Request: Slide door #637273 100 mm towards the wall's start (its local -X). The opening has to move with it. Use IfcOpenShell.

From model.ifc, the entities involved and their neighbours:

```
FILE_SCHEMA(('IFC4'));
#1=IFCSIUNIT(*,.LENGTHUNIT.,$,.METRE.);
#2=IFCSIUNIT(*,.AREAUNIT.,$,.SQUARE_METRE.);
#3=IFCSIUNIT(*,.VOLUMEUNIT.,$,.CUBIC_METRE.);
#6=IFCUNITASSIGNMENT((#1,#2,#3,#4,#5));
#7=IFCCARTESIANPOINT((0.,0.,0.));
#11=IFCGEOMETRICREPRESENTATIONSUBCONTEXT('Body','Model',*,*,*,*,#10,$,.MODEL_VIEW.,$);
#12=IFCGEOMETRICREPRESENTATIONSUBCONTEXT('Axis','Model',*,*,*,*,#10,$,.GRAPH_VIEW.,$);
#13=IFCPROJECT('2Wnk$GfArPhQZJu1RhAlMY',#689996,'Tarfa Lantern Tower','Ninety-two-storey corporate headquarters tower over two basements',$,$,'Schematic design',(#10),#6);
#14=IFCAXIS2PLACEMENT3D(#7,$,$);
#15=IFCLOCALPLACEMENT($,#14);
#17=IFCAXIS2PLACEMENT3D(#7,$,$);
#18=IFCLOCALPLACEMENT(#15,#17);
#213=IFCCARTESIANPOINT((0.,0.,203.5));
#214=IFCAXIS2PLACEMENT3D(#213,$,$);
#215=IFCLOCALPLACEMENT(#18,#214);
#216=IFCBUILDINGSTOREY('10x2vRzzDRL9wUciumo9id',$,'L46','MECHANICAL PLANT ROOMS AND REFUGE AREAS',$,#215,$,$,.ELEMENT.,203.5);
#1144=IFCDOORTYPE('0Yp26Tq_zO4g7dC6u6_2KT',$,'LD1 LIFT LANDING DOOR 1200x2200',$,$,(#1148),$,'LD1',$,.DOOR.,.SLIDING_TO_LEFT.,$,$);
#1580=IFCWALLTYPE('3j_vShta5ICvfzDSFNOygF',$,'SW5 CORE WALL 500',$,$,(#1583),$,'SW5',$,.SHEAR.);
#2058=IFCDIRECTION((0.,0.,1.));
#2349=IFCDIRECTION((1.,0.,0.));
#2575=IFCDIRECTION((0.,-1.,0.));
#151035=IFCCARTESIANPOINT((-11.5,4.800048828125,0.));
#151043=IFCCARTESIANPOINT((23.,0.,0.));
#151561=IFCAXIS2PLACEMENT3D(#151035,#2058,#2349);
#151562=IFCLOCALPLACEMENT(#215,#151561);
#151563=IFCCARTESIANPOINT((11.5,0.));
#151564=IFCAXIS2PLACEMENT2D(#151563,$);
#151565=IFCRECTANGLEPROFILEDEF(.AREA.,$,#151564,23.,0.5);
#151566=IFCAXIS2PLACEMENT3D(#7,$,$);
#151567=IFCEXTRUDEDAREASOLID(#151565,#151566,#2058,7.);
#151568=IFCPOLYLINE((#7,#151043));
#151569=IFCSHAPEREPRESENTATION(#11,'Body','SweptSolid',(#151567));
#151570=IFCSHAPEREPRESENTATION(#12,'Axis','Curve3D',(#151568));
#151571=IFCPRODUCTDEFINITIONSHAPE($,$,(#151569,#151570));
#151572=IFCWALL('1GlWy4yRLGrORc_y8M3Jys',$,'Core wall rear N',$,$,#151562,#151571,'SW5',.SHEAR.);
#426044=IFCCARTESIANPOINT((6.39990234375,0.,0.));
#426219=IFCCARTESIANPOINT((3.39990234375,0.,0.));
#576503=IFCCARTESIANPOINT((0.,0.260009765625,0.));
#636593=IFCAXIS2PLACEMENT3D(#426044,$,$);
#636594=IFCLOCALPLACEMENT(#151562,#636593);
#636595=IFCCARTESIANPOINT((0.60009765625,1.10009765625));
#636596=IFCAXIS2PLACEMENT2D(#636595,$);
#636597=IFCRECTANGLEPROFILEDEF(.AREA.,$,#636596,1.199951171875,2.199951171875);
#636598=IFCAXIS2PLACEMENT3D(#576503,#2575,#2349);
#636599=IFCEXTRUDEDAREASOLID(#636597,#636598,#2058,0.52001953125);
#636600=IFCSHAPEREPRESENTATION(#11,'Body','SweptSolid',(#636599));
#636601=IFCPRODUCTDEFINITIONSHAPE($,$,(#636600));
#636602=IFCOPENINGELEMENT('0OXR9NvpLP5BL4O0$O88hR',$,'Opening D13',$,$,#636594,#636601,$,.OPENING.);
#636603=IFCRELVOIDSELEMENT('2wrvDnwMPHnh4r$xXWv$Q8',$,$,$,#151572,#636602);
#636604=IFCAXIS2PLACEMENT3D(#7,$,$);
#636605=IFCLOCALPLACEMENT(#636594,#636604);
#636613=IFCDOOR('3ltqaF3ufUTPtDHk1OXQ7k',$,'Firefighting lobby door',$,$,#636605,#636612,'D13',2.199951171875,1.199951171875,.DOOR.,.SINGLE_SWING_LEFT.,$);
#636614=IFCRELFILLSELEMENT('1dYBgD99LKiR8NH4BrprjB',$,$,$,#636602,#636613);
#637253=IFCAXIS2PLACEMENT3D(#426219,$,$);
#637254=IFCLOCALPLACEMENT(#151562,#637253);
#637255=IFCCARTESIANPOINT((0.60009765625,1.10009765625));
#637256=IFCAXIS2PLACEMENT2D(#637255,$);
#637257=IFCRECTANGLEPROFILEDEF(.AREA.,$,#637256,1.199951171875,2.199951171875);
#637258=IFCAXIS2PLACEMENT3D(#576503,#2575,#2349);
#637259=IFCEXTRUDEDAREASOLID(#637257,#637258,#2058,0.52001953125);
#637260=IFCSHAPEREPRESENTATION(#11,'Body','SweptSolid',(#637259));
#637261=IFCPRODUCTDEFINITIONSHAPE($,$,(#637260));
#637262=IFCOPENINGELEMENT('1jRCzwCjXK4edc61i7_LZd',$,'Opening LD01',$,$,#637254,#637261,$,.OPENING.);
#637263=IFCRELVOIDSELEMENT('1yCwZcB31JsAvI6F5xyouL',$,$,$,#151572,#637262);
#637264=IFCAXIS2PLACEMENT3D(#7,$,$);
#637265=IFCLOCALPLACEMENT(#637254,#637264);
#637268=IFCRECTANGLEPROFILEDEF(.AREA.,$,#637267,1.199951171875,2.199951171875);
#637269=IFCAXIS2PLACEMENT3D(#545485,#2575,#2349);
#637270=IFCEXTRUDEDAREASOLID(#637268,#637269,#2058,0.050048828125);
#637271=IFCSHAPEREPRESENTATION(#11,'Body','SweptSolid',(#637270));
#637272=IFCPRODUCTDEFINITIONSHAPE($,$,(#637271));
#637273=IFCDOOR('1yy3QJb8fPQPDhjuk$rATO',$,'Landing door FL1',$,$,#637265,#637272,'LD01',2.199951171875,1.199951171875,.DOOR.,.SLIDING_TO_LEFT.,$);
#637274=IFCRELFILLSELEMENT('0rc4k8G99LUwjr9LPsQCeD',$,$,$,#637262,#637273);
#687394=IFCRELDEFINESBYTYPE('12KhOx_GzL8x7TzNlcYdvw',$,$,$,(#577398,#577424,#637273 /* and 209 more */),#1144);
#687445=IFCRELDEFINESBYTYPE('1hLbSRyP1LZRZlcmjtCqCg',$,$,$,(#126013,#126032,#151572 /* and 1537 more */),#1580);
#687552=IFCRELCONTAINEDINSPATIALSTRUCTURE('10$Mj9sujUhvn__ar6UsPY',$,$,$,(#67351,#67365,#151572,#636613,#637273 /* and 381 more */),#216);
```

```python
import ifcopenshell
import ifcopenshell.api.geometry
import ifcopenshell.util.placement
import ifcopenshell.util.unit

model = ifcopenshell.open("model.ifc")
unit_scale = ifcopenshell.util.unit.calculate_unit_scale(model)

door = model.by_guid("1yy3QJb8fPQPDhjuk$rATO")
opening = door.FillsVoids[0].RelatingOpeningElement
wall = opening.VoidsElements[0].RelatingBuildingElement

wall_matrix = ifcopenshell.util.placement.get_local_placement(wall.ObjectPlacement)
shift = wall_matrix[:3, 0] * -0.1 / unit_scale
before = ifcopenshell.util.placement.get_local_placement(door.ObjectPlacement)[:3, 3].copy()

# The door is placed relative to its opening, so it follows when the opening moves.
matrix = ifcopenshell.util.placement.get_local_placement(opening.ObjectPlacement)
matrix[:3, 3] += shift
ifcopenshell.api.geometry.edit_object_placement(
    model, product=opening, matrix=matrix, is_si=False, should_transform_children=True
)

after = ifcopenshell.util.placement.get_local_placement(door.ObjectPlacement)[:3, 3]
print("door moved by", (after - before).round(3) + 0.0)

model.write("model_updated.ifc")
```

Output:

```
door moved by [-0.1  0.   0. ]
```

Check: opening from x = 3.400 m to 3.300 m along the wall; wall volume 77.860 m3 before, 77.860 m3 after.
